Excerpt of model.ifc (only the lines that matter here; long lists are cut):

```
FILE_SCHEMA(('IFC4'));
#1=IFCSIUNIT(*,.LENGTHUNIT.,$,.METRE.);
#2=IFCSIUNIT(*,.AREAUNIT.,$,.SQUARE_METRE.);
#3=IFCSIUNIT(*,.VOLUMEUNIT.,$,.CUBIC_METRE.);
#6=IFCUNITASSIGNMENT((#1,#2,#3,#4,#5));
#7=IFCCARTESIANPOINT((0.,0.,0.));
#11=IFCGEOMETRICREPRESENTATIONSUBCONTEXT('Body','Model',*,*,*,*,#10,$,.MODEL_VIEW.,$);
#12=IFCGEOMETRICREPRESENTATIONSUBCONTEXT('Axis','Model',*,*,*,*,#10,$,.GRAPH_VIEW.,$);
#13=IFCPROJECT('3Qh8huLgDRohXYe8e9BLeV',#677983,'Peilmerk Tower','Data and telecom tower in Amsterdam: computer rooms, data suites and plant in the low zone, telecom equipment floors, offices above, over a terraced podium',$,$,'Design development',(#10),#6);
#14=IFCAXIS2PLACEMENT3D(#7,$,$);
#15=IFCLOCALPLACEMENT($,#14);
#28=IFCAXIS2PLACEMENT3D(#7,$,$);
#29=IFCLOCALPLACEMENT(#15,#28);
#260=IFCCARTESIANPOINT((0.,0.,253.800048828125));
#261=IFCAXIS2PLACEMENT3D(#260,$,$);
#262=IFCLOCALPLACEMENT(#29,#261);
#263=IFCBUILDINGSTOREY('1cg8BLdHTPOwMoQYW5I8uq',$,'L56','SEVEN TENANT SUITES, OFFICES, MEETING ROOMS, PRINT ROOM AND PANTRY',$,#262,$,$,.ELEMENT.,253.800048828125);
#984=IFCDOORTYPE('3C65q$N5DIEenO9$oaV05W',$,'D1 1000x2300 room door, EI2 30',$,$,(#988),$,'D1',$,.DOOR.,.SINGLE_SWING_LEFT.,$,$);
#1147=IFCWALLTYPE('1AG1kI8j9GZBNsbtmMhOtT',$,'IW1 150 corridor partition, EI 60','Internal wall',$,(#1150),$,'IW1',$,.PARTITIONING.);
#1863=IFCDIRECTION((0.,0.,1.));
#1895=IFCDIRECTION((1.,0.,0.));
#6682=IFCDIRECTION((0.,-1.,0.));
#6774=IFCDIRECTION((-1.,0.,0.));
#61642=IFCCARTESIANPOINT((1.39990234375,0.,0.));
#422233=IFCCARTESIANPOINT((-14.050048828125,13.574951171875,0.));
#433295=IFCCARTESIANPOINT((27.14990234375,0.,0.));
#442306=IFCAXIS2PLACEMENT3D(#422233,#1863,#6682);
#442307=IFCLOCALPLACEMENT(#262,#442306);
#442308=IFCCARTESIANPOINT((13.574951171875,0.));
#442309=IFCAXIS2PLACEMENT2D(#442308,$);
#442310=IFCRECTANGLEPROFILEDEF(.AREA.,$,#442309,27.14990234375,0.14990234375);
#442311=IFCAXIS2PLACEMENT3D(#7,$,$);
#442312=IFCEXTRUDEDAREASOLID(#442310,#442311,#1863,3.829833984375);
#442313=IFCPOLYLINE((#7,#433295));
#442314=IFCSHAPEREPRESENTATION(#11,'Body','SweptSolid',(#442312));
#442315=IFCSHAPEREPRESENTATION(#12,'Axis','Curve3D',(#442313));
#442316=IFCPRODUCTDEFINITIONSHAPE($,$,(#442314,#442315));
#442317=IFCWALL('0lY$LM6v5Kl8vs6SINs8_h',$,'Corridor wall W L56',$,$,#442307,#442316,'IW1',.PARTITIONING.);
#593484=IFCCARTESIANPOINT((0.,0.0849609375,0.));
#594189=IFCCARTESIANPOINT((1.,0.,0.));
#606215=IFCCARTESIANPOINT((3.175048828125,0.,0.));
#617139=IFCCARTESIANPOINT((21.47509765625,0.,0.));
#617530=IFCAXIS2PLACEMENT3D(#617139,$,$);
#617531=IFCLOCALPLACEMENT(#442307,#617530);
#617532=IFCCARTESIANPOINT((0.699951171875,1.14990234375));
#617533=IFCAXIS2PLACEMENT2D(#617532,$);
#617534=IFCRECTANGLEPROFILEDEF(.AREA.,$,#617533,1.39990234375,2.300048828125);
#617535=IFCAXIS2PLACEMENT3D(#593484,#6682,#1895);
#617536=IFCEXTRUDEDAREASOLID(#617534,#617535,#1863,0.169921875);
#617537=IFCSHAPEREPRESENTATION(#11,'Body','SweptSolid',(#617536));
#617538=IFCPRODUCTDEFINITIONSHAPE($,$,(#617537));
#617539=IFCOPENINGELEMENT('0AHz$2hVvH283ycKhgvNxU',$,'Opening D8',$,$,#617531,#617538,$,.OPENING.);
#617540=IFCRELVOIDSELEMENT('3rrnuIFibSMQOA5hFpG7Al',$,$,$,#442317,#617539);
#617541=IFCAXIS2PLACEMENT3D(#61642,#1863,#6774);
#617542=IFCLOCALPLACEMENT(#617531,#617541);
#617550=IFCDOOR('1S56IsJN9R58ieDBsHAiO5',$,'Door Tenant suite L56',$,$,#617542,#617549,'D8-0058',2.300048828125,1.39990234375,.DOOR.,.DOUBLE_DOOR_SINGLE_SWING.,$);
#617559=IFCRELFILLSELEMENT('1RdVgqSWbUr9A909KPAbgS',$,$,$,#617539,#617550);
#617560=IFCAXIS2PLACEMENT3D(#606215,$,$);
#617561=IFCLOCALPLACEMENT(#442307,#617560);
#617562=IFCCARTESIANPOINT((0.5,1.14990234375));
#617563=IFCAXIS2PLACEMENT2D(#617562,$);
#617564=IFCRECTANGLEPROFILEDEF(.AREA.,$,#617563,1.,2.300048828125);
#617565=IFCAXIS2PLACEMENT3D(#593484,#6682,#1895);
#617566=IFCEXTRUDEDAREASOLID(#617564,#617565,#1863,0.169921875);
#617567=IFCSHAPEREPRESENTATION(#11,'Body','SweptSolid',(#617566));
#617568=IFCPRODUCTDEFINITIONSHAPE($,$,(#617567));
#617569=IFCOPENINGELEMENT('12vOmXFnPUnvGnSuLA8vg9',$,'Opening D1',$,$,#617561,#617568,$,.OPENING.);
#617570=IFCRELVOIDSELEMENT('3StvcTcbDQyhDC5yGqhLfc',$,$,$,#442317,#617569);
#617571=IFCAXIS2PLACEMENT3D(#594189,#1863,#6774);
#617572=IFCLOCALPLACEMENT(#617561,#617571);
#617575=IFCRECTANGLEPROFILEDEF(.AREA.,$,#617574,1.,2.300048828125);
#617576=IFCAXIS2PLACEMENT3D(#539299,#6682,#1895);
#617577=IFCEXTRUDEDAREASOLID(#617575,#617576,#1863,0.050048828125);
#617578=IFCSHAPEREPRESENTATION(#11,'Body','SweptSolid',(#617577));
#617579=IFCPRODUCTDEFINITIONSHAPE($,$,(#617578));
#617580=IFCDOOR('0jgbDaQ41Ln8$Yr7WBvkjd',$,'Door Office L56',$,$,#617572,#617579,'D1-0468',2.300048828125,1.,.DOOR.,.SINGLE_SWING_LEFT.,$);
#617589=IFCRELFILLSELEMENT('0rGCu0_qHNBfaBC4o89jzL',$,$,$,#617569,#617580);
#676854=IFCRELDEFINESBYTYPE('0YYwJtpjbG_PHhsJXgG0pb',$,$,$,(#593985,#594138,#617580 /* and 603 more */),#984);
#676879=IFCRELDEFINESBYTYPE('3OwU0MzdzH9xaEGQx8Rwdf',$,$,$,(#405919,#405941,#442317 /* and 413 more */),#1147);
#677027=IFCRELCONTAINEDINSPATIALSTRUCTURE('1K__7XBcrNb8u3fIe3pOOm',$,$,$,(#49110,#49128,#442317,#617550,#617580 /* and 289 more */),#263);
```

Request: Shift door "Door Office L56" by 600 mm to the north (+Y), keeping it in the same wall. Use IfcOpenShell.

```python
import ifcopenshell
import ifcopenshell.api.geometry
import ifcopenshell.util.placement
import ifcopenshell.util.unit

model = ifcopenshell.open("model.ifc")
unit_scale = ifcopenshell.util.unit.calculate_unit_scale(model)

door = model.by_guid("0jgbDaQ41Ln8$Yr7WBvkjd")
opening = door.FillsVoids[0].RelatingOpeningElement
wall = opening.VoidsElements[0].RelatingBuildingElement

wall_matrix = ifcopenshell.util.placement.get_local_placement(wall.ObjectPlacement)
shift = wall_matrix[:3, 0] * -0.6 / unit_scale
before = ifcopenshell.util.placement.get_local_placement(door.ObjectPlacement)[:3, 3].copy()

# The door is placed relative to its opening, so it follows when the opening moves.
matrix = ifcopenshell.util.placement.get_local_placement(opening.ObjectPlacement)
matrix[:3, 3] += shift
ifcopenshell.api.geometry.edit_object_placement(
    model, product=opening, matrix=matrix, is_si=False, should_transform_children=True
)

after = ifcopenshell.util.placement.get_local_placement(door.ObjectPlacement)[:3, 3]
print("door moved by", (after - before).round(3) + 0.0)

model.write("model_updated.ifc")
```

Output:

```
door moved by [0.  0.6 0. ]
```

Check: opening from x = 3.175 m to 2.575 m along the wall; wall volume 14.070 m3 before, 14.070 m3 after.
